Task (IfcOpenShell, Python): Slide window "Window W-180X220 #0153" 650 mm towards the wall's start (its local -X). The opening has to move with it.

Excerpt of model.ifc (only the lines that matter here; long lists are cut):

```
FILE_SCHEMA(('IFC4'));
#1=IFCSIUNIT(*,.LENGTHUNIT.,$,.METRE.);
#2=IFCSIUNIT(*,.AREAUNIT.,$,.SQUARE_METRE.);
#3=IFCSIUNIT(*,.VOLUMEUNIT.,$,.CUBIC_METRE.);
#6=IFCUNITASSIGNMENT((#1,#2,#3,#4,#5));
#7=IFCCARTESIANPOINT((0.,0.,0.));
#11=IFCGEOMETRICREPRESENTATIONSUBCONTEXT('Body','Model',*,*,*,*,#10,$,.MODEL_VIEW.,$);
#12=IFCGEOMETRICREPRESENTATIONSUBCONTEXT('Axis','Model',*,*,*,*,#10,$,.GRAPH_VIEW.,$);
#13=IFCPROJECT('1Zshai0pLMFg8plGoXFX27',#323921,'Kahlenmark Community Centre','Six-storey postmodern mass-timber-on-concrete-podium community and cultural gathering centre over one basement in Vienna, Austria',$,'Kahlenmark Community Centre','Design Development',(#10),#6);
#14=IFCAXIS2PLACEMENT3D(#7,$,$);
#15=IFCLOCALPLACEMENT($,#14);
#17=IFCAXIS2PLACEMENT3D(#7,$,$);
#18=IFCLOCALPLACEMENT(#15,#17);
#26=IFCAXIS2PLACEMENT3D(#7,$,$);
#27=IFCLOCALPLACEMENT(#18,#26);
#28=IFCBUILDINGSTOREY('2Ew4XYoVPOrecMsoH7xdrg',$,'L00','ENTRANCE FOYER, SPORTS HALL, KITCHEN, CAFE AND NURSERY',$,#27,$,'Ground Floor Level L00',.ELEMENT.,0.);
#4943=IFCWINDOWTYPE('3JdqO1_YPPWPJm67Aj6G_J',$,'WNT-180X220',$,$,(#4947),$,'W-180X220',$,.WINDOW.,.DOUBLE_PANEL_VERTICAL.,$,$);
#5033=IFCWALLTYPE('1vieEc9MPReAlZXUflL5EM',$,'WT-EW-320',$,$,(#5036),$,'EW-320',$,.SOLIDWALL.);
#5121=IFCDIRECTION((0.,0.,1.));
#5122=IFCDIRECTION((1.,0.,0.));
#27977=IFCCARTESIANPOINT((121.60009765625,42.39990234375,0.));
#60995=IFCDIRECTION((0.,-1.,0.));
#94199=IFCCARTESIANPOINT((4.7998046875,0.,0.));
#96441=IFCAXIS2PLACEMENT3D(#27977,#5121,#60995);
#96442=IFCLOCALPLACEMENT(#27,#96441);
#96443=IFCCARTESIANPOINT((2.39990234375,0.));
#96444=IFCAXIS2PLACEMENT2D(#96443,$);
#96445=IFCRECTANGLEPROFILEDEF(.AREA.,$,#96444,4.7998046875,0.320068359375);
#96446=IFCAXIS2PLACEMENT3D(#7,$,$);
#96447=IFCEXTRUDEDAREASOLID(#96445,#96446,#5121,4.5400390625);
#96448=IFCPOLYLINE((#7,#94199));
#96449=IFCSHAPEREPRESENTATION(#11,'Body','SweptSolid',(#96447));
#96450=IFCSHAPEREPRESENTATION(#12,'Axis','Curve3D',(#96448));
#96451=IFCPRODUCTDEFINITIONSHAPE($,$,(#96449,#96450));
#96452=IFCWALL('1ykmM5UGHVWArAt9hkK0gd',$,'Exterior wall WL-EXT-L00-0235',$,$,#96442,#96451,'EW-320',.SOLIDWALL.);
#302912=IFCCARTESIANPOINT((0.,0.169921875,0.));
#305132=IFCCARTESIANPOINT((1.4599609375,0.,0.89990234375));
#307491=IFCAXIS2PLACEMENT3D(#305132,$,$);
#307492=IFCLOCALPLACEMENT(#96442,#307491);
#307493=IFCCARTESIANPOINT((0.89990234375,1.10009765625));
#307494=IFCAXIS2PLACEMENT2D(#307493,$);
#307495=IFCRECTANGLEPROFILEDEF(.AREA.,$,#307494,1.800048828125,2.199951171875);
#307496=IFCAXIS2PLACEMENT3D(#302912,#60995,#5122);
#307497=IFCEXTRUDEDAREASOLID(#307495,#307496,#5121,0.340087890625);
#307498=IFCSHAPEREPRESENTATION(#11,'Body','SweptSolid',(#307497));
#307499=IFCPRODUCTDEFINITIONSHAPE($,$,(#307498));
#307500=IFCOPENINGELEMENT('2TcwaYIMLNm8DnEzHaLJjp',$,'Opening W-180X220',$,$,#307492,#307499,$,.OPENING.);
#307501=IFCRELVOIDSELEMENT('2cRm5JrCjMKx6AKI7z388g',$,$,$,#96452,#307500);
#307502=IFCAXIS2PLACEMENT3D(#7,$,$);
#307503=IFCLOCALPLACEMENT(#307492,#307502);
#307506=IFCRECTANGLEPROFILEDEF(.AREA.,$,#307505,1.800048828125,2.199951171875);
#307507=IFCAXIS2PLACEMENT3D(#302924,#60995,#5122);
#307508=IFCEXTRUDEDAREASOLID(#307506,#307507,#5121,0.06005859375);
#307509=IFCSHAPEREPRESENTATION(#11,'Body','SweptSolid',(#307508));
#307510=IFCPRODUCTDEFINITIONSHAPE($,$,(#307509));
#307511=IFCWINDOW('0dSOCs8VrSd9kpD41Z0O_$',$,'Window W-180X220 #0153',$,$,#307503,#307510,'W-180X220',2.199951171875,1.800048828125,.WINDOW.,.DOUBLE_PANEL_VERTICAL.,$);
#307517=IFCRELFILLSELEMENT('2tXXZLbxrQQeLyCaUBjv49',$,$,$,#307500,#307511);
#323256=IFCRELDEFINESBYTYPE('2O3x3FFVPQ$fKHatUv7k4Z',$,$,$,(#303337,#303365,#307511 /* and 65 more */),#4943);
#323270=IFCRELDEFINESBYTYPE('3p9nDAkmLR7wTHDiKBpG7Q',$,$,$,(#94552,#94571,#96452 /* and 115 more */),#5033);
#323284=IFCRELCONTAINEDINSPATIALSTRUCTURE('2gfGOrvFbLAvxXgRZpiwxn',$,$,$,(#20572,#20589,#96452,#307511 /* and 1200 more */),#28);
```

```python
import ifcopenshell
import ifcopenshell.api.geometry
import ifcopenshell.util.placement
import ifcopenshell.util.unit

model = ifcopenshell.open("model.ifc")
unit_scale = ifcopenshell.util.unit.calculate_unit_scale(model)

window = model.by_guid("0dSOCs8VrSd9kpD41Z0O_$")
opening = window.FillsVoids[0].RelatingOpeningElement
wall = opening.VoidsElements[0].RelatingBuildingElement

wall_matrix = ifcopenshell.util.placement.get_local_placement(wall.ObjectPlacement)
shift = wall_matrix[:3, 0] * -0.65 / unit_scale
before = ifcopenshell.util.placement.get_local_placement(window.ObjectPlacement)[:3, 3].copy()

# The window is placed relative to its opening, so it follows when the opening moves.
matrix = ifcopenshell.util.placement.get_local_placement(opening.ObjectPlacement)
matrix[:3, 3] += shift
ifcopenshell.api.geometry.edit_object_placement(
    model, product=opening, matrix=matrix, is_si=False, should_transform_children=True
)

after = ifcopenshell.util.placement.get_local_placement(window.ObjectPlacement)[:3, 3]
print("window moved by", (after - before).round(3) + 0.0)

model.write("model_updated.ifc")
```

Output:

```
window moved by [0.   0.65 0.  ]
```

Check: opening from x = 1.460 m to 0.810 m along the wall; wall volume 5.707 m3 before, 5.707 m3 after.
